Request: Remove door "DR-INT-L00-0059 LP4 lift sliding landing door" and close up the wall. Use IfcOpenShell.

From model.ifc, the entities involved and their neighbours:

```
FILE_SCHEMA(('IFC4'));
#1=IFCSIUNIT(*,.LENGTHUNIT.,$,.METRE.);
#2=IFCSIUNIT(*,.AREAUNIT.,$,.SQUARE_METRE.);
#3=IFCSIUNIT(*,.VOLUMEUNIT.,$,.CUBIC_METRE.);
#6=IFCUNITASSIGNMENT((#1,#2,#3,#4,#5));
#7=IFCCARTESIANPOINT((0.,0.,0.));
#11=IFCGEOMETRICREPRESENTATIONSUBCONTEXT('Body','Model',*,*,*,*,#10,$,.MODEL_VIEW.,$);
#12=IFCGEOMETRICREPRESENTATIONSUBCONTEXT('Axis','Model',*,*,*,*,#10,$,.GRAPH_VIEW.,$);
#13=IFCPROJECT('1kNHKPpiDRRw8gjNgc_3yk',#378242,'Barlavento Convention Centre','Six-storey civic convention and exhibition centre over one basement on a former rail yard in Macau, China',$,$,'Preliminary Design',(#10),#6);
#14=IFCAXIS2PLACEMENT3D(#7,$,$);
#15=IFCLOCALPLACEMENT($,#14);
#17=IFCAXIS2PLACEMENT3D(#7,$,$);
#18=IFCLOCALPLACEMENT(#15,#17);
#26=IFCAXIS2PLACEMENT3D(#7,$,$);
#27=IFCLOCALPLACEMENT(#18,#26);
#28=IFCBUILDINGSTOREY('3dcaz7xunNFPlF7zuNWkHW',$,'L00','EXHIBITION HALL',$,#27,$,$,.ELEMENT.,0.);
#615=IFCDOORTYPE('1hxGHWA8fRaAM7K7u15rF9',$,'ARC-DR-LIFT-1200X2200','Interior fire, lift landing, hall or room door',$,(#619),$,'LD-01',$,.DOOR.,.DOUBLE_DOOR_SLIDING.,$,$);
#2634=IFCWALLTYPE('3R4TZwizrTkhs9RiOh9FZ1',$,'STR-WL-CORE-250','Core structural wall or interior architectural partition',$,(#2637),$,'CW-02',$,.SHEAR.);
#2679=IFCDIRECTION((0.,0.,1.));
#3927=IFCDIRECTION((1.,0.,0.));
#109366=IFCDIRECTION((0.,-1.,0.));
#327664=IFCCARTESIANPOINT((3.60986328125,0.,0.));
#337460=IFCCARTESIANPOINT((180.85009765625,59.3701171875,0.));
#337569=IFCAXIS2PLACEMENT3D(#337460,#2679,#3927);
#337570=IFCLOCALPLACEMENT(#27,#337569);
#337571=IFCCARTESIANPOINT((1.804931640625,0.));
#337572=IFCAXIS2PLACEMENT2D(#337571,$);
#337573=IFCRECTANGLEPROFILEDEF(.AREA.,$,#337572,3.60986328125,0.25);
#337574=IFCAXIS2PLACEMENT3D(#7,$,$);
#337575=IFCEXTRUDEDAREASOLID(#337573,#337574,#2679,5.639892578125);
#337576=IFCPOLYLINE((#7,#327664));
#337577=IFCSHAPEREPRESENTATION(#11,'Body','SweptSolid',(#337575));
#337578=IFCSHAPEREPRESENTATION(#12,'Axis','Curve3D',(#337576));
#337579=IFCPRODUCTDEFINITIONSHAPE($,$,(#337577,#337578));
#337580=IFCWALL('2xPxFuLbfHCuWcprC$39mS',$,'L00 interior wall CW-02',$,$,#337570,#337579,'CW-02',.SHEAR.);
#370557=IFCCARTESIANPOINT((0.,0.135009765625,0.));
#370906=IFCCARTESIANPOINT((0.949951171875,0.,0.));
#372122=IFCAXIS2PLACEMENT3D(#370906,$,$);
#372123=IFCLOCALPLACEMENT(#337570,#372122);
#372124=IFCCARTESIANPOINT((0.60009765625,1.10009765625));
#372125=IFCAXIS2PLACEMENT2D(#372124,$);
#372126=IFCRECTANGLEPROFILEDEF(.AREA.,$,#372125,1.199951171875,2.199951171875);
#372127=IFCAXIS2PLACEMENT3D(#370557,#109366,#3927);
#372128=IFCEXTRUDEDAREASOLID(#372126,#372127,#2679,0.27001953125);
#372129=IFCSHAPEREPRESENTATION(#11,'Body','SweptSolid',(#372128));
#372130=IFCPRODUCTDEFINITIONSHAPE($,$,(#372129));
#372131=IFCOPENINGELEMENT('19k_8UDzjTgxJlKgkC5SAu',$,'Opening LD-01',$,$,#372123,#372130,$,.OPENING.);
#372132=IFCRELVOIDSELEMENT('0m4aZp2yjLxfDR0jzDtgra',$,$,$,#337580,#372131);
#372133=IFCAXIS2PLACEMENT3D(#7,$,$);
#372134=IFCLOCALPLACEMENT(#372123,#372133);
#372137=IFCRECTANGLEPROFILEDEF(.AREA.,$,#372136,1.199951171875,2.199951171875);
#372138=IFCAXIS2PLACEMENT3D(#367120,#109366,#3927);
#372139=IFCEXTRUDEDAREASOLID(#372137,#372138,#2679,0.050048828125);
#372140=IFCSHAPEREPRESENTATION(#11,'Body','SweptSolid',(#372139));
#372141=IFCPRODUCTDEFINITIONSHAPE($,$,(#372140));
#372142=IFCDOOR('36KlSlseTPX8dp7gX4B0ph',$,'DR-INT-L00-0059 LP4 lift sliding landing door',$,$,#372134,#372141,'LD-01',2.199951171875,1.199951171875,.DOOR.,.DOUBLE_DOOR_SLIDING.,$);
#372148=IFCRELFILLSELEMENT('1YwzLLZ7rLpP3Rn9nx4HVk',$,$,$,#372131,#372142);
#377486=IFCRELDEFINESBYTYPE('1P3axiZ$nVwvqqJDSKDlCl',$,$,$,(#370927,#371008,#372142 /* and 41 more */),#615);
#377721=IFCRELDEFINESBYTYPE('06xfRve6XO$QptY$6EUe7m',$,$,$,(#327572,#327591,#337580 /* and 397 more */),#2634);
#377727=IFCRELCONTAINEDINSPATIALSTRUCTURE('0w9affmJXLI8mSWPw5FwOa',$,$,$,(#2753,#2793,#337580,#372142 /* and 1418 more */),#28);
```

```python
import ifcopenshell
import ifcopenshell.api.feature
import ifcopenshell.api.root
import ifcopenshell.geom
import ifcopenshell.util.shape

model = ifcopenshell.open("model.ifc")
settings = ifcopenshell.geom.settings()


def volume(element):
    """Net volume in cubic metres, openings subtracted."""
    shape = ifcopenshell.geom.create_shape(settings, element)
    return ifcopenshell.util.shape.get_volume(shape.geometry)


door = model.by_guid("36KlSlseTPX8dp7gX4B0ph")
opening = door.FillsVoids[0].RelatingOpeningElement
wall = opening.VoidsElements[0].RelatingBuildingElement
before = volume(wall)

ifcopenshell.api.root.remove_product(model, product=door)
ifcopenshell.api.feature.remove_feature(model, feature=opening)

after = volume(wall)

print(f"wall volume {before:.3f} -> {after:.3f} m3")

model.write("model_rev.ifc")
```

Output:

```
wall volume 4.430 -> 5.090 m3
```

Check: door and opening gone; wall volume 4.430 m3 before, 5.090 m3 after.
